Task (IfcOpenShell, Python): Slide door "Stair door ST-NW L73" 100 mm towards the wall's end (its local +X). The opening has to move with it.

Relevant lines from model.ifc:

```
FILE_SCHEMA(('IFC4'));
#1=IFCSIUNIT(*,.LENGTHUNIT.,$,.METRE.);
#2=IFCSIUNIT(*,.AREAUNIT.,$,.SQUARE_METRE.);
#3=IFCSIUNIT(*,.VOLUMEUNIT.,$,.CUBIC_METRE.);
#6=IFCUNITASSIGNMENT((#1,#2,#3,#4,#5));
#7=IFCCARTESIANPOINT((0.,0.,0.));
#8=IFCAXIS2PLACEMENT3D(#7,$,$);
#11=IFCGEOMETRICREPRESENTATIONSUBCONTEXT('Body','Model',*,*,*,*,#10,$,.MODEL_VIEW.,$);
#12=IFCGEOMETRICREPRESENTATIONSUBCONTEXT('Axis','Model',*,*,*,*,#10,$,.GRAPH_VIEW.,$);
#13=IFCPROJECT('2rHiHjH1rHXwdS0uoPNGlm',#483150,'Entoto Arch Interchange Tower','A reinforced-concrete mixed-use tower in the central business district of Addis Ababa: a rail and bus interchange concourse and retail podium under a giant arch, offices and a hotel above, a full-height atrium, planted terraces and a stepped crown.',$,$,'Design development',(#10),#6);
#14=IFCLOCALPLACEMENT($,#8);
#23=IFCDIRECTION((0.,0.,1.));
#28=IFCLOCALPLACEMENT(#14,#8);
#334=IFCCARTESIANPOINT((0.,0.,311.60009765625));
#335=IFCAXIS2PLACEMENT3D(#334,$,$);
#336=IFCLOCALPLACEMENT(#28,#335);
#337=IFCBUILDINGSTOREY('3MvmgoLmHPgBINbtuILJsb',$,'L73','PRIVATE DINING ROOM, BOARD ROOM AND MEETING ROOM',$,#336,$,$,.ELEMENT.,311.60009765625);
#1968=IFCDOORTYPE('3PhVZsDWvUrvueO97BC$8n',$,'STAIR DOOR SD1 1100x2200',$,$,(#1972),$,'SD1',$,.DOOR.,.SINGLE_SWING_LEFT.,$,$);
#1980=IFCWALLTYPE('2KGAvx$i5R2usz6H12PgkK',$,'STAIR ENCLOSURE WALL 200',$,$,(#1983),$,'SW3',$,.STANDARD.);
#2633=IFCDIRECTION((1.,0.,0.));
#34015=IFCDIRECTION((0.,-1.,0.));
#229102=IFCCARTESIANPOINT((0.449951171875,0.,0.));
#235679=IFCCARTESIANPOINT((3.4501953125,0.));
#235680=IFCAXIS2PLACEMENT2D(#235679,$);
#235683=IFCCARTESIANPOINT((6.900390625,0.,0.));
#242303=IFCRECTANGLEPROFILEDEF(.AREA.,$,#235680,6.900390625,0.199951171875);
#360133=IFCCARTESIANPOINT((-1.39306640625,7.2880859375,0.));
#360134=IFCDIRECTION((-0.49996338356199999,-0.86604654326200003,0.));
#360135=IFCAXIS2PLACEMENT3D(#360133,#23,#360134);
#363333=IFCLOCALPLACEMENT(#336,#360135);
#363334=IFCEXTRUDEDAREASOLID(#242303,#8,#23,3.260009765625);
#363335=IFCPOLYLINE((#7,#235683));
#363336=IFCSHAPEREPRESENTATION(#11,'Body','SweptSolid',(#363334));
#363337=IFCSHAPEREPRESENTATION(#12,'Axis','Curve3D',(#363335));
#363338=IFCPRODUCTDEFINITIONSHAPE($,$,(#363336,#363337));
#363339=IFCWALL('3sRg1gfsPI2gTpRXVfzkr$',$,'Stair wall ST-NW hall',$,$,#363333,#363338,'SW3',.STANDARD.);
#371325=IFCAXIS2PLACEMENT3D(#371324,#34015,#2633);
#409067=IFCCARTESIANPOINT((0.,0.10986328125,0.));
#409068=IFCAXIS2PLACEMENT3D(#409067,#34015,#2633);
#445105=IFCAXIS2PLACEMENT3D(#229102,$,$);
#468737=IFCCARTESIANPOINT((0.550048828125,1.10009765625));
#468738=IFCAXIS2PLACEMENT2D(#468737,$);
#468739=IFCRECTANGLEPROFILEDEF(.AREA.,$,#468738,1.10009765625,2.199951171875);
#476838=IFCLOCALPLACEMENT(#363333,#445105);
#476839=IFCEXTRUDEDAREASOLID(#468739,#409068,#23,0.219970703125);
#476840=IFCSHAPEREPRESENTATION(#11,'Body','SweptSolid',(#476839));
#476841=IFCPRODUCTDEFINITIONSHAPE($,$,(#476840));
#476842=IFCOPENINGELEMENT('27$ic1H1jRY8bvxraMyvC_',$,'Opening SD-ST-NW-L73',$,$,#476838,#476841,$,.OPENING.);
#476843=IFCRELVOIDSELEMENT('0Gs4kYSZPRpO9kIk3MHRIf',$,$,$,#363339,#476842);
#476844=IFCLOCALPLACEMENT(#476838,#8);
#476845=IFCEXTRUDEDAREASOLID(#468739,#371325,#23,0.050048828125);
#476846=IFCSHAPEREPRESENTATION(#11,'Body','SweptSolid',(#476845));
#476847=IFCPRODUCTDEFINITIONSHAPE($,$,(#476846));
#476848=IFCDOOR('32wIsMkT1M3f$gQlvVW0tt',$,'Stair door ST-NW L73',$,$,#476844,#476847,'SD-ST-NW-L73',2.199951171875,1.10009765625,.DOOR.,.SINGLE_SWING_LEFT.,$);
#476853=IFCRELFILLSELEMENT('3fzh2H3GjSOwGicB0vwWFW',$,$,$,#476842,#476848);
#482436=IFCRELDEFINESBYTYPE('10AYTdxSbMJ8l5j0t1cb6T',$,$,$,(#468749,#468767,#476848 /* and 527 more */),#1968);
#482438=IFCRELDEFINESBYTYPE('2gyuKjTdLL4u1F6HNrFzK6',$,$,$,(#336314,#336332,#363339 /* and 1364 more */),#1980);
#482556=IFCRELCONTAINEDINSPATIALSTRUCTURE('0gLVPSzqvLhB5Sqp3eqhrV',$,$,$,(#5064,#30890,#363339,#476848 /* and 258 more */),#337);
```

```python
import ifcopenshell
import ifcopenshell.api.geometry
import ifcopenshell.util.placement
import ifcopenshell.util.unit

model = ifcopenshell.open("model.ifc")
unit_scale = ifcopenshell.util.unit.calculate_unit_scale(model)

door = model.by_id(476848)
opening = door.FillsVoids[0].RelatingOpeningElement
wall = opening.VoidsElements[0].RelatingBuildingElement

wall_matrix = ifcopenshell.util.placement.get_local_placement(wall.ObjectPlacement)
shift = wall_matrix[:3, 0] * 0.1 / unit_scale
before = ifcopenshell.util.placement.get_local_placement(door.ObjectPlacement)[:3, 3].copy()

# The door is placed relative to its opening, so it follows when the opening moves.
matrix = ifcopenshell.util.placement.get_local_placement(opening.ObjectPlacement)
matrix[:3, 3] += shift
ifcopenshell.api.geometry.edit_object_placement(
    model, product=opening, matrix=matrix, is_si=False, should_transform_children=True
)

after = ifcopenshell.util.placement.get_local_placement(door.ObjectPlacement)[:3, 3]
print("door moved by", (after - before).round(3) + 0.0)

model.write("model_edited.ifc")
```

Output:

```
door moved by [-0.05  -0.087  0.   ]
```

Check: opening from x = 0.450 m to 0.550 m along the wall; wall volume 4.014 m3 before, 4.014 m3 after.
